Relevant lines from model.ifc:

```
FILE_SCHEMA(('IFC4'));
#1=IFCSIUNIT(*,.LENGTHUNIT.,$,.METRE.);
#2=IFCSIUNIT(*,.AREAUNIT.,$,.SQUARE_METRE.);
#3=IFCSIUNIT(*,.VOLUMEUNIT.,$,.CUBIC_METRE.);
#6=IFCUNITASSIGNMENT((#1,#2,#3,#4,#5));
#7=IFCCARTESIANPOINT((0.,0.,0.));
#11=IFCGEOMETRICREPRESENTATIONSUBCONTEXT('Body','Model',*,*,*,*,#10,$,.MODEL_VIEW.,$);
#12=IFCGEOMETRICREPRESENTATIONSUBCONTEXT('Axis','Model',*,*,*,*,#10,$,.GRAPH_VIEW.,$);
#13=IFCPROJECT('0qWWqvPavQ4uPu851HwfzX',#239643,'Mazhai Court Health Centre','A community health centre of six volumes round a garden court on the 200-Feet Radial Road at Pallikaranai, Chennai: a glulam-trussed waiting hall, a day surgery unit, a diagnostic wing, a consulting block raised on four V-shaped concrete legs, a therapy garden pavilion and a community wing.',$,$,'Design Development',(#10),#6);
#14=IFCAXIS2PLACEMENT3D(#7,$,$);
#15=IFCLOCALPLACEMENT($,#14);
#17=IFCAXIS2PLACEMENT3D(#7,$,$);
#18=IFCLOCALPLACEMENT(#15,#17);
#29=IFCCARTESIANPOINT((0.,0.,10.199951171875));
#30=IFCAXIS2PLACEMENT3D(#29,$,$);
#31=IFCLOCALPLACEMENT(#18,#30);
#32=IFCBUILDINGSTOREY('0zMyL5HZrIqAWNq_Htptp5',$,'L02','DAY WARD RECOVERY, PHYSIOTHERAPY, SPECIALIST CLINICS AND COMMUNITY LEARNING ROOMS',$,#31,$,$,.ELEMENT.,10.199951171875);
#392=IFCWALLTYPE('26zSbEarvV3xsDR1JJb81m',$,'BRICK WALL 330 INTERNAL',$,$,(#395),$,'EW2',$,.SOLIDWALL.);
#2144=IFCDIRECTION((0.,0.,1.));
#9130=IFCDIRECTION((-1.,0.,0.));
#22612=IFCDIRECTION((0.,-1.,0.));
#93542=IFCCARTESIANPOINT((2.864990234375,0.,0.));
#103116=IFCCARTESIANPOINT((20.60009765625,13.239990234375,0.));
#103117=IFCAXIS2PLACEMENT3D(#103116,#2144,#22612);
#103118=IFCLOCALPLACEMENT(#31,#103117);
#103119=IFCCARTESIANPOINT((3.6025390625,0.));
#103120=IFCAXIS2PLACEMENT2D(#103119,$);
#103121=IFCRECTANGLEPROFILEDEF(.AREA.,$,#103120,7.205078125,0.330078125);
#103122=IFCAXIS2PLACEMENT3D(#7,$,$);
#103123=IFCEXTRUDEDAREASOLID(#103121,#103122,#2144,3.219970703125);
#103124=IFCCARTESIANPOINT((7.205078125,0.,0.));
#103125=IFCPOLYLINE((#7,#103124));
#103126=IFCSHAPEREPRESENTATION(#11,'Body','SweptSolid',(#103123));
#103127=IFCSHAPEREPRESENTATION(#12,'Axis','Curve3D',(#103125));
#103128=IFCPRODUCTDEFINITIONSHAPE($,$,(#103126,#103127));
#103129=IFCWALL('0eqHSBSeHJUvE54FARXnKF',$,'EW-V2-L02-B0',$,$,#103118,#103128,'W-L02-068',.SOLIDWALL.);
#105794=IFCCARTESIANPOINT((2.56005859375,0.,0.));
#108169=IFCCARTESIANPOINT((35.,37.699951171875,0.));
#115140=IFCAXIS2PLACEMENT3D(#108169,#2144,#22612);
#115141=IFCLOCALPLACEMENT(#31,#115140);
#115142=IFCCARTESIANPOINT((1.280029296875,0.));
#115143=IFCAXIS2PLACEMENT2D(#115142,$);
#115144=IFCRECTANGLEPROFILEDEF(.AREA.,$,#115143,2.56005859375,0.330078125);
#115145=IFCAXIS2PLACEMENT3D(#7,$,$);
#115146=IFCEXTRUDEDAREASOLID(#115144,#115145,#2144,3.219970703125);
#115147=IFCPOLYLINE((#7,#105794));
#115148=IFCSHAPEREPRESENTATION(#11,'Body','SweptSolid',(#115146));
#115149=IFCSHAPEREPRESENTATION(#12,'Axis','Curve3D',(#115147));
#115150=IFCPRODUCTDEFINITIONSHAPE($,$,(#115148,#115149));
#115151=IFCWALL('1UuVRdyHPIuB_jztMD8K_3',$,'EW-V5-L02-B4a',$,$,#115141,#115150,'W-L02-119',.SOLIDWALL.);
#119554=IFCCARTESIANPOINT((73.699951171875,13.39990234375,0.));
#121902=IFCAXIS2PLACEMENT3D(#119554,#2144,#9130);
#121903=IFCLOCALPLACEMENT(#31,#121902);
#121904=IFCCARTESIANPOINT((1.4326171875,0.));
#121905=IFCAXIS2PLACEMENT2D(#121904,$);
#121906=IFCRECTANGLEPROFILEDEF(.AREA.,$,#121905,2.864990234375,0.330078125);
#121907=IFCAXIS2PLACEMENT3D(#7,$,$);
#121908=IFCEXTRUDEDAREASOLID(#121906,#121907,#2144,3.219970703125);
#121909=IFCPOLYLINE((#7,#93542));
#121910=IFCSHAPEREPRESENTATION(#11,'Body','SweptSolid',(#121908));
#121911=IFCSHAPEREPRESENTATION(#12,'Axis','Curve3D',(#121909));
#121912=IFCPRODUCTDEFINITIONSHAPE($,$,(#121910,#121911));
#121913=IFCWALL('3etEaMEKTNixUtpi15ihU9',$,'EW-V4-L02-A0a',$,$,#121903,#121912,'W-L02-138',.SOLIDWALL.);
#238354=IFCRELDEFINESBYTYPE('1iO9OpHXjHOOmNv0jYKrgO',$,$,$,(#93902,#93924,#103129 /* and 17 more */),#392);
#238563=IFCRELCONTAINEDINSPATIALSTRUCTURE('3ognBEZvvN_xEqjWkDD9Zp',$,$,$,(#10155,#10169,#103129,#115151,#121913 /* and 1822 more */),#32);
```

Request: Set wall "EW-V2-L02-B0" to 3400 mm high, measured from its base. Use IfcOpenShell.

```python
import ifcopenshell
import ifcopenshell.geom
import ifcopenshell.util.representation
import ifcopenshell.util.shape
import ifcopenshell.util.unit

model = ifcopenshell.open("model.ifc")
unit_scale = ifcopenshell.util.unit.calculate_unit_scale(model)
settings = ifcopenshell.geom.settings()


def volume(element):
    """Net volume in cubic metres, openings subtracted."""
    shape = ifcopenshell.geom.create_shape(settings, element)
    return ifcopenshell.util.shape.get_volume(shape.geometry)


wall = model.by_guid("0eqHSBSeHJUvE54FARXnKF")
before = volume(wall)

body = ifcopenshell.util.representation.get_representation(wall, "Model", "Body")
solid = body.Items[0]
old_height = solid.Depth
solid.Depth = 3.4 / unit_scale
after = volume(wall)

print(f"height {old_height:g} -> {solid.Depth:g}, volume {before:.3f} -> {after:.3f} m3")

model.write("model_v2.ifc")
```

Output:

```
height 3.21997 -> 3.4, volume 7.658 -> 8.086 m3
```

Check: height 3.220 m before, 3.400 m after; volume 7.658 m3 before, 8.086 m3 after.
